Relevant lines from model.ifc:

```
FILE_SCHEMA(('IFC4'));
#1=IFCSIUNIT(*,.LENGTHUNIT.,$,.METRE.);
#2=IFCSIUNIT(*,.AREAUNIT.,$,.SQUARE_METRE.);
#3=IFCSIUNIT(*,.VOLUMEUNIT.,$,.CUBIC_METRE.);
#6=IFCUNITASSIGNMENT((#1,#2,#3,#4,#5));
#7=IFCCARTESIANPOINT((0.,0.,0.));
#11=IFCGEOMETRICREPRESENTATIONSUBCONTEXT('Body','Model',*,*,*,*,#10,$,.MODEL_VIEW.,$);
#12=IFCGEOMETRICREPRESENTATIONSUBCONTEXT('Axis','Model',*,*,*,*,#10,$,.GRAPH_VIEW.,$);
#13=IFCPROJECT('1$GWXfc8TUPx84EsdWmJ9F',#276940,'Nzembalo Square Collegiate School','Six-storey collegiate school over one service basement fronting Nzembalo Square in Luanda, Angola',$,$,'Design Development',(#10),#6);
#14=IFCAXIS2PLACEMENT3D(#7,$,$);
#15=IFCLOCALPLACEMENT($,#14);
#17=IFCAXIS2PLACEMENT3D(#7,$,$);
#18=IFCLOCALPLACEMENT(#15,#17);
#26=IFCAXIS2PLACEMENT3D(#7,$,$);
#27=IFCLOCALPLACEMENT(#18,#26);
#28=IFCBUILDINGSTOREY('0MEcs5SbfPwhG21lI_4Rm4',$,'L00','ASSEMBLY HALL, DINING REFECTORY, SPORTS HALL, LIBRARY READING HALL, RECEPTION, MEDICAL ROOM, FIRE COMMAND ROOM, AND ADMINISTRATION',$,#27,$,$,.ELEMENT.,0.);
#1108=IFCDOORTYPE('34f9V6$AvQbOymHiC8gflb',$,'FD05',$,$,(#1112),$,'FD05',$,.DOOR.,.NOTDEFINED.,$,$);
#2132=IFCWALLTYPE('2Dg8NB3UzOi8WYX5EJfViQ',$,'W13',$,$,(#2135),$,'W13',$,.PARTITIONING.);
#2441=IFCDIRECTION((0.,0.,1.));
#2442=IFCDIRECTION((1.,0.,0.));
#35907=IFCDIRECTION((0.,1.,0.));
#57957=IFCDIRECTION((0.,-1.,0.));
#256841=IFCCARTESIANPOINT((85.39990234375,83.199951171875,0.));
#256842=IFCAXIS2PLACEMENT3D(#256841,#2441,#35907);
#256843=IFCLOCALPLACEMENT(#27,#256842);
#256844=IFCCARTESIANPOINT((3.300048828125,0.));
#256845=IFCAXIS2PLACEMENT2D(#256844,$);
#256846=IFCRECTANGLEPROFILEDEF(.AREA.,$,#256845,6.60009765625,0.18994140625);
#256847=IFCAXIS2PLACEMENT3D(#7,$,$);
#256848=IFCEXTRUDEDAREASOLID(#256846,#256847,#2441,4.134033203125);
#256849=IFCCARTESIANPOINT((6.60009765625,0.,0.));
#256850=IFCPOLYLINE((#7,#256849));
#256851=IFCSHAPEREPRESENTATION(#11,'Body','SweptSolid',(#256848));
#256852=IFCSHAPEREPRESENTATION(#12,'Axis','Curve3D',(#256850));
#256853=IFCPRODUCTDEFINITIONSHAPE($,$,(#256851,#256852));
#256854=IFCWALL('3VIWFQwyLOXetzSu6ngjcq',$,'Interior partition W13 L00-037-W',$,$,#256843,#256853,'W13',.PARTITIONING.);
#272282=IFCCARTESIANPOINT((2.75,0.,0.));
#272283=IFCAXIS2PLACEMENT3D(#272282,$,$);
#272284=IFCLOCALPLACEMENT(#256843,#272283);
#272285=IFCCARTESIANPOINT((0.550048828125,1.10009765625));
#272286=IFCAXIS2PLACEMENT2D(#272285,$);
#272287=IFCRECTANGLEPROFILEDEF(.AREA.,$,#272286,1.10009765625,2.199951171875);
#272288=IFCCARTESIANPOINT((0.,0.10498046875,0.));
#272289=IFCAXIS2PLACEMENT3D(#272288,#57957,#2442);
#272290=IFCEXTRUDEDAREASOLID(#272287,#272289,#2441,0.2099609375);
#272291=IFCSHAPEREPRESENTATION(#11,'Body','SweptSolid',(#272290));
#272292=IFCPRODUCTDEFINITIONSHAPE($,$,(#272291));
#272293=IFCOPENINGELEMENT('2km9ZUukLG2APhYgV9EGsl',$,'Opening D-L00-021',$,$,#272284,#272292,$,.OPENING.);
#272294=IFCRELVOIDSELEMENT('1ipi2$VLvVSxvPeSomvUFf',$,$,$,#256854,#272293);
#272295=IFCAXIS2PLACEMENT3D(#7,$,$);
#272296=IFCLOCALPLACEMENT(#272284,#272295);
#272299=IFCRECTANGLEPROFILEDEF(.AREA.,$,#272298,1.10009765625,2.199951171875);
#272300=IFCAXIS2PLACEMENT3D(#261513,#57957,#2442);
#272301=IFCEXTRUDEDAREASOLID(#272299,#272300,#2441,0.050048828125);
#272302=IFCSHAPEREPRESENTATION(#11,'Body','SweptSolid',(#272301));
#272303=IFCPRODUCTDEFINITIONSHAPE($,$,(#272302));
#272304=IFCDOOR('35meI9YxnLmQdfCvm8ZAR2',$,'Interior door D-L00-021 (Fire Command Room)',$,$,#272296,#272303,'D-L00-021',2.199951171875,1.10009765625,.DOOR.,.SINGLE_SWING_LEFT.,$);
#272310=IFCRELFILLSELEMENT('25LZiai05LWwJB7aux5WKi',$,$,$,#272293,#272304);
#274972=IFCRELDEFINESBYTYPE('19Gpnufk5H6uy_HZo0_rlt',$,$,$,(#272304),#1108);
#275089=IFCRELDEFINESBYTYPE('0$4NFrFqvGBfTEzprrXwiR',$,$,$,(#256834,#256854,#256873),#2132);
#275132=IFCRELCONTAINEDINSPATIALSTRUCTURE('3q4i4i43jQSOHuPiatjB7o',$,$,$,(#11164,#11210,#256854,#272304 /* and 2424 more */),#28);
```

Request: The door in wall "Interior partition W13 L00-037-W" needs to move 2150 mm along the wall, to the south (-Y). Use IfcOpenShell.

```python
import ifcopenshell
import ifcopenshell.api.geometry
import ifcopenshell.util.placement
import ifcopenshell.util.unit

model = ifcopenshell.open("model.ifc")
unit_scale = ifcopenshell.util.unit.calculate_unit_scale(model)

door = model.by_guid("35meI9YxnLmQdfCvm8ZAR2")
opening = door.FillsVoids[0].RelatingOpeningElement
wall = opening.VoidsElements[0].RelatingBuildingElement

wall_matrix = ifcopenshell.util.placement.get_local_placement(wall.ObjectPlacement)
shift = wall_matrix[:3, 0] * -2.15 / unit_scale
before = ifcopenshell.util.placement.get_local_placement(door.ObjectPlacement)[:3, 3].copy()

# The door is placed relative to its opening, so it follows when the opening moves.
matrix = ifcopenshell.util.placement.get_local_placement(opening.ObjectPlacement)
matrix[:3, 3] += shift
ifcopenshell.api.geometry.edit_object_placement(
    model, product=opening, matrix=matrix, is_si=False, should_transform_children=True
)

after = ifcopenshell.util.placement.get_local_placement(door.ObjectPlacement)[:3, 3]
print("door moved by", (after - before).round(3) + 0.0)

model.write("model_v2.ifc")
```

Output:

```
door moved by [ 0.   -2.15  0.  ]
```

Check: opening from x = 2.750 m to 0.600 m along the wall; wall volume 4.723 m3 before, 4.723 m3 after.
